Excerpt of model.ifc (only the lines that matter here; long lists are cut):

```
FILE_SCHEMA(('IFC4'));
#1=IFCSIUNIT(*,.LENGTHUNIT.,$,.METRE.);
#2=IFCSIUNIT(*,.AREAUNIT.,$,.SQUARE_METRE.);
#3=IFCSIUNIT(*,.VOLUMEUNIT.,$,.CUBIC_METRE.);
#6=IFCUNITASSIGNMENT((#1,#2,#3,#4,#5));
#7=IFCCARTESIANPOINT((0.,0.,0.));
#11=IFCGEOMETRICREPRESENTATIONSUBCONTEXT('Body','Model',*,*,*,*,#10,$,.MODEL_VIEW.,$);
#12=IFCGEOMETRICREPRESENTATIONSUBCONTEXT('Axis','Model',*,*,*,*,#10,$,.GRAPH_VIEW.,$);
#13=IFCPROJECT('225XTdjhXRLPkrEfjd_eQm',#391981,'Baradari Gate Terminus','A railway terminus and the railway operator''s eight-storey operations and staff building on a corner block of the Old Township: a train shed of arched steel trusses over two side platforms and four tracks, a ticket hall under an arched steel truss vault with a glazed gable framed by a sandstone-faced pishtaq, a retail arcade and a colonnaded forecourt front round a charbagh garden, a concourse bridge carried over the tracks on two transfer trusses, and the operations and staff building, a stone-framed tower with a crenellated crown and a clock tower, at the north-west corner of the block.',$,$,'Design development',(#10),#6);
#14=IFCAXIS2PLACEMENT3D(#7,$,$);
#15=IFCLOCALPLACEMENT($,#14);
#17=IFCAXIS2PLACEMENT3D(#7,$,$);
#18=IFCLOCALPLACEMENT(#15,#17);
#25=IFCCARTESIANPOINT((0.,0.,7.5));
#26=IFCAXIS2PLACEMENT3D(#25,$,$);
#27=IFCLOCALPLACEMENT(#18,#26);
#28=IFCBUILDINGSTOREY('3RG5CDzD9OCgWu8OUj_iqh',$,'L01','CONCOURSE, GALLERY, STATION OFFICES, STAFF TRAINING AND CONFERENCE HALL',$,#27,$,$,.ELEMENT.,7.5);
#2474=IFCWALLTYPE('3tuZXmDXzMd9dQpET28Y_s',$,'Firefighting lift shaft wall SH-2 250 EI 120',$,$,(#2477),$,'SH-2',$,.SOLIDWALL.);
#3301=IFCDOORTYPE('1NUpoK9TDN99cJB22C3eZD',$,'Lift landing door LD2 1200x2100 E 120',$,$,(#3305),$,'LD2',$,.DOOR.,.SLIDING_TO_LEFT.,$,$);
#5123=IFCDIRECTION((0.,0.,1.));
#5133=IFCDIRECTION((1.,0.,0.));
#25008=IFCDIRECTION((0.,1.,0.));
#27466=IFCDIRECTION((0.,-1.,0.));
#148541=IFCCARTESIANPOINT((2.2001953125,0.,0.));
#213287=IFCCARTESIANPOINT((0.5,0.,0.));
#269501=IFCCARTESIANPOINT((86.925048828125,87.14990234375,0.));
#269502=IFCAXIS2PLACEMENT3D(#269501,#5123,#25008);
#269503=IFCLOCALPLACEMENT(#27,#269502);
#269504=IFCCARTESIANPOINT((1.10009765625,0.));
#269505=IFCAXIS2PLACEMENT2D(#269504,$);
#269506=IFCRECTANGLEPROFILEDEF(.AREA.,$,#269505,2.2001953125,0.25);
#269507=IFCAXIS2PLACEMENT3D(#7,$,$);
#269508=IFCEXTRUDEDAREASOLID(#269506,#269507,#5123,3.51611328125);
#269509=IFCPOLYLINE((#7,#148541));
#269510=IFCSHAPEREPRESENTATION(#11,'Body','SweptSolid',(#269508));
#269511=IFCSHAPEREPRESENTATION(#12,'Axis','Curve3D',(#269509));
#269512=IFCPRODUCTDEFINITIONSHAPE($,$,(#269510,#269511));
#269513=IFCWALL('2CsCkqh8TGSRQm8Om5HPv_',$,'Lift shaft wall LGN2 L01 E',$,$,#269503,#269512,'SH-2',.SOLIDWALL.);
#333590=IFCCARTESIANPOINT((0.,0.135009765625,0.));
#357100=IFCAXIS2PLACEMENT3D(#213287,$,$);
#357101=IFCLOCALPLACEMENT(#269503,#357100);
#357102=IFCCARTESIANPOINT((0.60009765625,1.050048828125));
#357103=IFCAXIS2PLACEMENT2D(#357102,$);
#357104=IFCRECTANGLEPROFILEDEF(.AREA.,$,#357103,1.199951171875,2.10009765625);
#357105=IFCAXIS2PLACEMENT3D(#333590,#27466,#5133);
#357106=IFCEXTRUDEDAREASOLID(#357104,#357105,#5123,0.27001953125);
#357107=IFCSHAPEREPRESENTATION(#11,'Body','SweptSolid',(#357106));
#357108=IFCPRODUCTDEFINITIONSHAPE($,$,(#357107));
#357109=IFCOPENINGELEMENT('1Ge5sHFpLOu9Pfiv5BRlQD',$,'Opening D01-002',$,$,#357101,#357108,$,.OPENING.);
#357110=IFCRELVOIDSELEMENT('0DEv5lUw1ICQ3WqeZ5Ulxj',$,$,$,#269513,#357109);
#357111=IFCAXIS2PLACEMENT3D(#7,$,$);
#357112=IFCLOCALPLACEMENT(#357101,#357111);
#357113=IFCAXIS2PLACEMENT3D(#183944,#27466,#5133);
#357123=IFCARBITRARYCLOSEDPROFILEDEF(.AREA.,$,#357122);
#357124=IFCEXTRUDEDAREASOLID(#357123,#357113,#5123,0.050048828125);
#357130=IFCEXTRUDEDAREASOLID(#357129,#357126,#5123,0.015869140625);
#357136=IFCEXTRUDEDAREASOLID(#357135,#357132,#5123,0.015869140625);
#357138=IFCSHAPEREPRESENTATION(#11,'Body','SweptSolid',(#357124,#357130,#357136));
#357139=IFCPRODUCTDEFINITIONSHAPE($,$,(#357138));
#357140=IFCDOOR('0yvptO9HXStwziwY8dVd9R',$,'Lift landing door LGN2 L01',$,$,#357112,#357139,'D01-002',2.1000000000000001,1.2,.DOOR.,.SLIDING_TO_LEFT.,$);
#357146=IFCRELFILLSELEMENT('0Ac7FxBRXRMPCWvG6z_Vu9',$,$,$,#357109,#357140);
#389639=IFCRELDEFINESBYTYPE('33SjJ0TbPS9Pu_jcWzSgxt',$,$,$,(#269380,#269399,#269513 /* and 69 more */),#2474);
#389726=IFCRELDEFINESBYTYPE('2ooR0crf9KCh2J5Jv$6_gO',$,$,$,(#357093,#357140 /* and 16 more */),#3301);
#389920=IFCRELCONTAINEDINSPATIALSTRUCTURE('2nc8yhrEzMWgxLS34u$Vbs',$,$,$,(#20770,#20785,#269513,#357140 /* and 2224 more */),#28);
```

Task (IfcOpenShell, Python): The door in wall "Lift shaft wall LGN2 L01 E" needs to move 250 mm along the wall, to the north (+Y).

```python
import ifcopenshell
import ifcopenshell.api.geometry
import ifcopenshell.util.placement

model = ifcopenshell.open("model.ifc")

door = model.by_guid("0yvptO9HXStwziwY8dVd9R")
opening = door.FillsVoids[0].RelatingOpeningElement
wall = opening.VoidsElements[0].RelatingBuildingElement

wall_matrix = ifcopenshell.util.placement.get_local_placement(wall.ObjectPlacement)
shift = wall_matrix[:3, 0] * 0.25
before = ifcopenshell.util.placement.get_local_placement(door.ObjectPlacement)[:3, 3].copy()

# The door is placed relative to its opening, so it follows when the opening moves.
matrix = ifcopenshell.util.placement.get_local_placement(opening.ObjectPlacement)
matrix[:3, 3] += shift
ifcopenshell.api.geometry.edit_object_placement(
    model, product=opening, matrix=matrix, is_si=False, should_transform_children=True
)

after = ifcopenshell.util.placement.get_local_placement(door.ObjectPlacement)[:3, 3]
print("door moved by", (after - before).round(3) + 0.0)

model.write("model_edited.ifc")
```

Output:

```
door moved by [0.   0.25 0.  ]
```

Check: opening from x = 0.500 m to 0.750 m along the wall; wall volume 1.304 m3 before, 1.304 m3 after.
